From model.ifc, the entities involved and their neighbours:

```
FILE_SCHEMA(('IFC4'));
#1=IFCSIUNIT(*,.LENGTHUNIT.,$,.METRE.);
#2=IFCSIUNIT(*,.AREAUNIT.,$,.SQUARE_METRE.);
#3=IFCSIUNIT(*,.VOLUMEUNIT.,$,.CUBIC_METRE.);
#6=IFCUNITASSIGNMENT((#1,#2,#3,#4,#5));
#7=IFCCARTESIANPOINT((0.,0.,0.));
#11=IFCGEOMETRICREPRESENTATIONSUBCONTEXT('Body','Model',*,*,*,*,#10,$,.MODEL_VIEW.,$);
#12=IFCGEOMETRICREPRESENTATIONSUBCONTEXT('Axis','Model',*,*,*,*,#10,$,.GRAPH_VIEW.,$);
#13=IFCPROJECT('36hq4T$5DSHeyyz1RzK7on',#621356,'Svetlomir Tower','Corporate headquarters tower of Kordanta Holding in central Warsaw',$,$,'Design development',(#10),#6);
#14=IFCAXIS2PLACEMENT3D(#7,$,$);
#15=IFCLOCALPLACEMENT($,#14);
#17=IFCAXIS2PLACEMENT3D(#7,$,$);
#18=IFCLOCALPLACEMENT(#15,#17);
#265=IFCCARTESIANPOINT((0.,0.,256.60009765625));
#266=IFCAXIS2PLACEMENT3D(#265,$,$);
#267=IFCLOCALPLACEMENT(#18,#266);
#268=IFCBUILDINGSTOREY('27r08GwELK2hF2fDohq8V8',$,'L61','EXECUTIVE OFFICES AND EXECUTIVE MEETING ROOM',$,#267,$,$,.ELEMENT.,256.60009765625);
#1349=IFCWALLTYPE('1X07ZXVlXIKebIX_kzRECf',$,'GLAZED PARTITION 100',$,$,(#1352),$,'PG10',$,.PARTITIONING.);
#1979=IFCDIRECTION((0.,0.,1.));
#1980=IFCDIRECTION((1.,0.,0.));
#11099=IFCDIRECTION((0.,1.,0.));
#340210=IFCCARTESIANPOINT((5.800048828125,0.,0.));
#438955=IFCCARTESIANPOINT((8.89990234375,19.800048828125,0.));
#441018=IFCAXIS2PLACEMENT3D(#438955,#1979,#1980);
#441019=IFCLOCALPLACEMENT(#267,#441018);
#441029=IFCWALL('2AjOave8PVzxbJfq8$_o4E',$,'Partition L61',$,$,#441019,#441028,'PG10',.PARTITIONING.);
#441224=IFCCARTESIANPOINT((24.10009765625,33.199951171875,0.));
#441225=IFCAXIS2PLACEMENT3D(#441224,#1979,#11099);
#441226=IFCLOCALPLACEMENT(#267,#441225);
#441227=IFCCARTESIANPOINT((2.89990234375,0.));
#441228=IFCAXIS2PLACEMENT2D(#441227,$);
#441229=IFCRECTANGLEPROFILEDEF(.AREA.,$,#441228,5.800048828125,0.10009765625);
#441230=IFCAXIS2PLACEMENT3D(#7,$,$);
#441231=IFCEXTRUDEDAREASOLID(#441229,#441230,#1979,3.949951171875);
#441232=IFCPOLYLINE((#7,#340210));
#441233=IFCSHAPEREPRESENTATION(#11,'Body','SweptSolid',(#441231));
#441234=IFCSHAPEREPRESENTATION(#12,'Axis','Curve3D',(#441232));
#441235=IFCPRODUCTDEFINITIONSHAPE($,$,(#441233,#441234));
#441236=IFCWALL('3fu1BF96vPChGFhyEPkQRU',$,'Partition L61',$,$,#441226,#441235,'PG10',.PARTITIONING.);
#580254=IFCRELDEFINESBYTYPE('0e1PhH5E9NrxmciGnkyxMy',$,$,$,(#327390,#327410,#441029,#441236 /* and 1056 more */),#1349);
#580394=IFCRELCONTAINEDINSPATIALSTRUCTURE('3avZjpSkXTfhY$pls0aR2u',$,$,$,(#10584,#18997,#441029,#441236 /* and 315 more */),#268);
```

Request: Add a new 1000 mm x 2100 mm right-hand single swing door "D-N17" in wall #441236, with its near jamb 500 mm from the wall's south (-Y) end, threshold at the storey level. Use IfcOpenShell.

```python
import numpy as np
import ifcopenshell
import ifcopenshell.api.feature
import ifcopenshell.api.geometry
import ifcopenshell.api.root
import ifcopenshell.api.spatial
import ifcopenshell.geom
import ifcopenshell.util.element
import ifcopenshell.util.placement
import ifcopenshell.util.representation
import ifcopenshell.util.shape
import ifcopenshell.util.unit

model = ifcopenshell.open("model.ifc")
unit_scale = ifcopenshell.util.unit.calculate_unit_scale(model)
settings = ifcopenshell.geom.settings()


def volume(element):
    """Net volume in cubic metres, openings subtracted."""
    shape = ifcopenshell.geom.create_shape(settings, element)
    return ifcopenshell.util.shape.get_volume(shape.geometry)


wall = model.by_guid("3fu1BF96vPChGFhyEPkQRU")
storey = ifcopenshell.util.element.get_container(wall, ifc_class="IfcBuildingStorey")
context = ifcopenshell.util.representation.get_context(model, "Model", "Body", "MODEL_VIEW")
before = volume(wall)

width, height, from_end, sill = 1, 2.1, 0.5, 0.0  # metres

# The wall runs along its own X axis, and the end named is its -X end.
wall_shape = ifcopenshell.geom.create_shape(settings, wall)
x, y, z = ifcopenshell.util.shape.get_vertices(wall_shape.geometry).T
start = x.min() + from_end
face, thickness = float(y.min()), float(y.max() - y.min())
wall_matrix = ifcopenshell.util.placement.get_local_placement(wall.ObjectPlacement)
level = ifcopenshell.util.placement.get_local_placement(storey.ObjectPlacement)[2, 3]


def in_wall(x, y):
    """Placement at x, y metres in the wall's axes, at sill height."""
    matrix = wall_matrix.copy()
    matrix[:, 3] = wall_matrix @ np.array([x / unit_scale, y / unit_scale, 0.0, 1.0])
    matrix[2, 3] = level + sill / unit_scale
    return matrix


# Opening: a box that overshoots both wall faces by 50 mm.
opening = ifcopenshell.api.root.create_entity(model, ifc_class="IfcOpeningElement", predefined_type="OPENING")
box = ifcopenshell.api.geometry.add_wall_representation(
    model, context=context, length=width, height=height, thickness=thickness + 0.1
)
ifcopenshell.api.geometry.assign_representation(model, product=opening, representation=box)
ifcopenshell.api.geometry.edit_object_placement(model, product=opening, matrix=in_wall(start, face - 0.05), is_si=False)
ifcopenshell.api.feature.add_feature(model, feature=opening, element=wall)

door = ifcopenshell.api.root.create_entity(model, ifc_class="IfcDoor", name="D-N17", predefined_type="DOOR")
door.OverallWidth, door.OverallHeight = width / unit_scale, height / unit_scale
door.OperationType = "SINGLE_SWING_RIGHT"
body = ifcopenshell.api.geometry.add_door_representation(
    model,
    context=context,
    overall_width=door.OverallWidth,
    overall_height=door.OverallHeight,
    operation_type="SINGLE_SWING_RIGHT",
    lining_properties={"LiningDepth": thickness / unit_scale, "ThresholdDepth": thickness / unit_scale},
)
ifcopenshell.api.geometry.assign_representation(model, product=door, representation=body)
ifcopenshell.api.spatial.assign_container(model, products=[door], relating_structure=storey)
ifcopenshell.api.feature.add_filling(model, opening=opening, element=door)

# The lining spans the wall, so the door starts at the wall face.
ifcopenshell.api.geometry.edit_object_placement(model, product=door, matrix=in_wall(start, face), is_si=False)

after = volume(wall)

print(f"wall volume {before:.3f} -> {after:.3f} m3")

model.write("model_updated.ifc")
```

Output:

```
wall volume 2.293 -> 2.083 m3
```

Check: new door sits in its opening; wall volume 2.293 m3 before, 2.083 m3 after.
